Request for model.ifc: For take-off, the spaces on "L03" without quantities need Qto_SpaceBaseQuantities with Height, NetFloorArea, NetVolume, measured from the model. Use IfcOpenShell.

First a look at what the model holds.

```python
import ifcopenshell
import ifcopenshell.util.element
import ifcopenshell.util.unit

model = ifcopenshell.open("model.ifc")
print(model.schema)
for unit_type in ("LENGTHUNIT", "AREAUNIT", "VOLUMEUNIT"):
    print(unit_type, ifcopenshell.util.unit.calculate_unit_scale(model, unit_type))
storey = next(s for s in model.by_type("IfcBuildingStorey") if s.Name == "L03")
spaces = [e for e in ifcopenshell.util.element.get_decomposition(storey) if e.is_a("IfcSpace")]
for e in sorted(spaces, key=lambda e: e.id()):
    print(e.id(), e.is_a(), e.Name, list(ifcopenshell.util.element.get_psets(e, qtos_only=True)), sep=" | ")
```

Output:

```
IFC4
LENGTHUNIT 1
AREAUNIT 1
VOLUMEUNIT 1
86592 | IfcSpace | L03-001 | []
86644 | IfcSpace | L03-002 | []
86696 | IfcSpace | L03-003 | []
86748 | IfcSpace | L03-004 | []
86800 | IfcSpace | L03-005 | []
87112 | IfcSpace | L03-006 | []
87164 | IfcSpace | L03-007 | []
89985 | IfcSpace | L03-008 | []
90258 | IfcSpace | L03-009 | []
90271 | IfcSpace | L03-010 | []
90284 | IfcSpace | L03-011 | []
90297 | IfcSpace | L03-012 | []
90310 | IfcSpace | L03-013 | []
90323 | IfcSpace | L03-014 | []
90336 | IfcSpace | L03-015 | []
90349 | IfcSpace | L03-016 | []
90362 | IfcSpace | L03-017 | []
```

```python
import ifcopenshell
import ifcopenshell.api.pset
import ifcopenshell.geom
import ifcopenshell.util.element
import ifcopenshell.util.shape
import ifcopenshell.util.unit

model = ifcopenshell.open("model.ifc")
unit_scale = ifcopenshell.util.unit.calculate_unit_scale(model)
area_scale = ifcopenshell.util.unit.calculate_unit_scale(model, "AREAUNIT")
volume_scale = ifcopenshell.util.unit.calculate_unit_scale(model, "VOLUMEUNIT")
settings = ifcopenshell.geom.settings()

storey = next(s for s in model.by_type("IfcBuildingStorey") if s.Name == "L03")
spaces = [e for e in ifcopenshell.util.element.get_decomposition(storey) if e.is_a("IfcSpace")]

for e in sorted(spaces, key=lambda e: e.id()):
    if ifcopenshell.util.element.get_psets(e, qtos_only=True, should_inherit=False):
        continue
    # Geometry comes back in metres, in the element's own axes.
    shape = ifcopenshell.geom.create_shape(settings, e)
    values = {
        "Height": ifcopenshell.util.shape.get_z(shape.geometry) / unit_scale,
        "NetFloorArea": ifcopenshell.util.shape.get_footprint_area(shape.geometry) / area_scale,
        "NetVolume": ifcopenshell.util.shape.get_volume(shape.geometry) / volume_scale,
    }
    qto = ifcopenshell.api.pset.add_qto(model, product=e, name="Qto_SpaceBaseQuantities")
    ifcopenshell.api.pset.edit_qto(model, qto=qto, properties=values)
    print(e.id(), {k: round(v, 3) for k, v in values.items()})

model.write("model_updated.ifc")
```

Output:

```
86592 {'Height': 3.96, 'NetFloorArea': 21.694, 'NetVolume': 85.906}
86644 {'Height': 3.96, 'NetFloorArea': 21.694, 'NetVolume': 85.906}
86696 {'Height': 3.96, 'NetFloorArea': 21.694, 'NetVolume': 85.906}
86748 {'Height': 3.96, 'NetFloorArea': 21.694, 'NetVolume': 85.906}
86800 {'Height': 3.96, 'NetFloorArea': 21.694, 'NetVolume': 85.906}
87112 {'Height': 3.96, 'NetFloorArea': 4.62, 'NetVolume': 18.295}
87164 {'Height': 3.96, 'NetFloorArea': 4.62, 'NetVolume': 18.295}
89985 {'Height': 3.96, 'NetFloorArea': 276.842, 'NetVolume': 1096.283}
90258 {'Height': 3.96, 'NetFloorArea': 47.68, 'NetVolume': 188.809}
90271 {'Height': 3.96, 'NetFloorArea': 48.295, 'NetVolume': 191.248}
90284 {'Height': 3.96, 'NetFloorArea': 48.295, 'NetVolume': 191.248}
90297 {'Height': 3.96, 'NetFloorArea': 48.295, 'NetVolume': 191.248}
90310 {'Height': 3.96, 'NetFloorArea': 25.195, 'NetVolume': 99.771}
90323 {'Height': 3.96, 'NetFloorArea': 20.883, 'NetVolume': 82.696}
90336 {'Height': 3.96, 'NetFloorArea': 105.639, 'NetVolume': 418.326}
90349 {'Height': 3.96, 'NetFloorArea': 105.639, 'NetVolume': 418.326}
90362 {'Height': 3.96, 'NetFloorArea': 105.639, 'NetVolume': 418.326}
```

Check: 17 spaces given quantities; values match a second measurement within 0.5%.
